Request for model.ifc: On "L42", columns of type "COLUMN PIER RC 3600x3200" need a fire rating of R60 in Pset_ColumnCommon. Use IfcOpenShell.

First a look at what the model holds.

```python
import ifcopenshell
import ifcopenshell.util.element

model = ifcopenshell.open("model.ifc")
print(model.schema)
storey = next(s for s in model.by_type("IfcBuildingStorey") if s.Name == "L42")
columns = [e for e in ifcopenshell.util.element.get_decomposition(storey) if e.is_a("IfcColumn")]
seen = {}
for e in columns:
    element_type = ifcopenshell.util.element.get_type(e)
    key = (element_type.Name if element_type != e and element_type else None, ifcopenshell.util.element.get_pset(e, "Pset_ColumnCommon", "FireRating"))
    seen[key] = seen.get(key, 0) + 1
for (name, value), count in sorted(seen.items(), key=str):
    print(count, "x", name, "|", value)
```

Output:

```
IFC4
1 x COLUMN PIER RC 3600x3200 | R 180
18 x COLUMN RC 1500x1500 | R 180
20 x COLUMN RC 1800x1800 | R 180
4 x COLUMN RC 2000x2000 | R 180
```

```python
import ifcopenshell
import ifcopenshell.api.pset
import ifcopenshell.util.element

model = ifcopenshell.open("model.ifc")

storey = next(s for s in model.by_type("IfcBuildingStorey") if s.Name == "L42")
columns = [e for e in ifcopenshell.util.element.get_decomposition(storey) if e.is_a("IfcColumn")]

count = 0
for e in columns:
    element_type = ifcopenshell.util.element.get_type(e)
    if element_type in (None, e) or element_type.Name != "COLUMN PIER RC 3600x3200":
        continue
    found = ifcopenshell.util.element.get_pset(e, "Pset_ColumnCommon", should_inherit=False)
    if found:
        pset = model.by_id(found["id"])
        if len(ifcopenshell.util.element.get_elements_by_pset(pset)) > 1:
            pset = ifcopenshell.api.pset.unshare_pset(model, products=[e], pset=pset)[0]
    else:
        pset = ifcopenshell.api.pset.add_pset(model, product=e, name="Pset_ColumnCommon")
    ifcopenshell.api.pset.edit_pset(model, pset=pset, properties={"FireRating": "R60"})
    count += 1

print(count, "columns updated")

model.write("model_v2.ifc")
```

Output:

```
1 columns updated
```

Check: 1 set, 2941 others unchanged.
